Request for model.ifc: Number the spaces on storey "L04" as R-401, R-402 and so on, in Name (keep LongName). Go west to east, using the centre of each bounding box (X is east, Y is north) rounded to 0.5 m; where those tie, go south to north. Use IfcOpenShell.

First a look at what the model holds.

```python
import ifcopenshell
import ifcopenshell.util.element
import ifcopenshell.util.placement

model = ifcopenshell.open("model.ifc")
print(model.schema)
storey = next(s for s in model.by_type("IfcBuildingStorey") if s.Name == "L04")
spaces = [e for e in ifcopenshell.util.element.get_decomposition(storey) if e.is_a("IfcSpace")]
for e in sorted(spaces, key=lambda e: e.id()):
    origin = ifcopenshell.util.placement.get_local_placement(e.ObjectPlacement)[:3, 3]
    print(e.id(), e.Name, e.LongName, origin.round(2) + 0.0, sep=" | ")
```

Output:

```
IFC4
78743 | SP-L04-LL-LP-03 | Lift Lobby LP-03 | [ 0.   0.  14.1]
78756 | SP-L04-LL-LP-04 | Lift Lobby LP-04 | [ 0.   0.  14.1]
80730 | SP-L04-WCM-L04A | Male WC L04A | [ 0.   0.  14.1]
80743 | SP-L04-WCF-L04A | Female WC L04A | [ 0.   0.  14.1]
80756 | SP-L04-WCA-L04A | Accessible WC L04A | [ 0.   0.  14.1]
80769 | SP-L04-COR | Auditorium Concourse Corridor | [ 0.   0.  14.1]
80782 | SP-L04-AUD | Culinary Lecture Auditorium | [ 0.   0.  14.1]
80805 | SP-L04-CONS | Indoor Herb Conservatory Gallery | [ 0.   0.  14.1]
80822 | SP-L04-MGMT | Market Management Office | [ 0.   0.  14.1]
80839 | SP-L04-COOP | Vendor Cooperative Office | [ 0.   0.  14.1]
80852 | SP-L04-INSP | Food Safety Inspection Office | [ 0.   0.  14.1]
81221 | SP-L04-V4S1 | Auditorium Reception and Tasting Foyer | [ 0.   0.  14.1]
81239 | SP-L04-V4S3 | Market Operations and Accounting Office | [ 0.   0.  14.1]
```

```python
import ifcopenshell
import ifcopenshell.geom
import ifcopenshell.util.element
import ifcopenshell.util.shape

model = ifcopenshell.open("model.ifc")
settings = ifcopenshell.geom.settings()
settings.set("use-world-coords", True)


def centre(element):
    shape = ifcopenshell.geom.create_shape(settings, element)
    return ifcopenshell.util.shape.get_bbox_centroid(shape.geometry)


storey = next(s for s in model.by_type("IfcBuildingStorey") if s.Name == "L04")
spaces = [e for e in ifcopenshell.util.element.get_decomposition(storey) if e.is_a("IfcSpace")]

# Insertion points can sit at a corner or the storey origin, so sort by the geometry (in metres).
centres = {e: centre(e) for e in spaces}
spaces.sort(key=lambda e: (round(centres[e][0] / 0.5), centres[e][1]))

for i, e in enumerate(spaces, start=1):
    number = f"R-4{i:02d}"
    e.Name = number
    print(e.id(), number)

model.write("model_updated.ifc")
```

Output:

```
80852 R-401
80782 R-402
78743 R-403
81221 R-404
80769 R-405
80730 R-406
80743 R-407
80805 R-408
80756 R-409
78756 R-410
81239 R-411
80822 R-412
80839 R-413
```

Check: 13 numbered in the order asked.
